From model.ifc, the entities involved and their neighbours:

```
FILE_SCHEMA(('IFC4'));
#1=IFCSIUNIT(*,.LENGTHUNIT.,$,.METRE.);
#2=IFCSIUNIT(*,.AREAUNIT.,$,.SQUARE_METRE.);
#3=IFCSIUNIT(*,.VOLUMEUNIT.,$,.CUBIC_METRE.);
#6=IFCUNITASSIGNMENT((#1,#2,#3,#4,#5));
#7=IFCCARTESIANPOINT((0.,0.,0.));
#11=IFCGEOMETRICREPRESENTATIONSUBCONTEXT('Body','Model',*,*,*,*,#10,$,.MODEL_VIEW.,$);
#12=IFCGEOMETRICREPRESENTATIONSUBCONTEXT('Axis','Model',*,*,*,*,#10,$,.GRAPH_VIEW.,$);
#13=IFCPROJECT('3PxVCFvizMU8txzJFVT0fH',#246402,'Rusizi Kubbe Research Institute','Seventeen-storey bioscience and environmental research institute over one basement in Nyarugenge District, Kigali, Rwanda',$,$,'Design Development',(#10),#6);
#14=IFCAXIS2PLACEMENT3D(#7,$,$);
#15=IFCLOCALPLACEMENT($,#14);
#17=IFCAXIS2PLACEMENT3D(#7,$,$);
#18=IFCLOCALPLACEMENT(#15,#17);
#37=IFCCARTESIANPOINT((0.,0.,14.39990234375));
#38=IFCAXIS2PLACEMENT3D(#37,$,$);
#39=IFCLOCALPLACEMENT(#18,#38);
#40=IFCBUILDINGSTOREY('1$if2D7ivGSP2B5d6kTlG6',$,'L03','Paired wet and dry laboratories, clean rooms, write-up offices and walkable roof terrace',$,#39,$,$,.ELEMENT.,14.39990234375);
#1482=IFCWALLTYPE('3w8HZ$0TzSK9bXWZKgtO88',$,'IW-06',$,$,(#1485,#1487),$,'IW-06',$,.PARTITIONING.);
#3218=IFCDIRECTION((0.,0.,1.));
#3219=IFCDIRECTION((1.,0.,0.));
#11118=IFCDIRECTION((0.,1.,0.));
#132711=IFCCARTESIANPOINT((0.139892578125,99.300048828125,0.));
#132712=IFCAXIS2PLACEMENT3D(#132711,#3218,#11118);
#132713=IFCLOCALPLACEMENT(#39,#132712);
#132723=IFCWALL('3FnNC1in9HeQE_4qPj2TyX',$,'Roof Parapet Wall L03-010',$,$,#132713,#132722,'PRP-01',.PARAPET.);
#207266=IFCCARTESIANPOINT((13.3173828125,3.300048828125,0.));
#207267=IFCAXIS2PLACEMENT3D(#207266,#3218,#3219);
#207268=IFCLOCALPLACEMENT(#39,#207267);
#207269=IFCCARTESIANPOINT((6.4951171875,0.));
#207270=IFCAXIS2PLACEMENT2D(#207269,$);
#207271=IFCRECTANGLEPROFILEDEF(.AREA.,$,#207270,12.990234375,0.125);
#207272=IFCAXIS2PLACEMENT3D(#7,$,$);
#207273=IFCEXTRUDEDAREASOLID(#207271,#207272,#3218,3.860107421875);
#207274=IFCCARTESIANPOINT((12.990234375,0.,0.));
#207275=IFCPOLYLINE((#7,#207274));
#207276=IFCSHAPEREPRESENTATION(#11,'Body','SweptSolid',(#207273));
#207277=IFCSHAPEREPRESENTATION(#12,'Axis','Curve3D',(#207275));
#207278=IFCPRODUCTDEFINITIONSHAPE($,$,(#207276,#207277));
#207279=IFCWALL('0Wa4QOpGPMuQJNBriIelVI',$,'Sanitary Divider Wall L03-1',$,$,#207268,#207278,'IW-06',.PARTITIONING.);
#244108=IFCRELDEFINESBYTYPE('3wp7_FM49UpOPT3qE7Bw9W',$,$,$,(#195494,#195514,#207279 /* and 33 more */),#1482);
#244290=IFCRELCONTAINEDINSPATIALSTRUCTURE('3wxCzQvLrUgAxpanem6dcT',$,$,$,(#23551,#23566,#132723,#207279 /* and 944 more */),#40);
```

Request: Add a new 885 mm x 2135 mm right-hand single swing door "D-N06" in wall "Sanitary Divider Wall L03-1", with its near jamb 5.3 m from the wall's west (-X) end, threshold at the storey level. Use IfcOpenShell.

```python
import numpy as np
import ifcopenshell
import ifcopenshell.api.feature
import ifcopenshell.api.geometry
import ifcopenshell.api.root
import ifcopenshell.api.spatial
import ifcopenshell.geom
import ifcopenshell.util.element
import ifcopenshell.util.placement
import ifcopenshell.util.representation
import ifcopenshell.util.shape
import ifcopenshell.util.unit

model = ifcopenshell.open("model.ifc")
unit_scale = ifcopenshell.util.unit.calculate_unit_scale(model)
settings = ifcopenshell.geom.settings()


def volume(element):
    """Net volume in cubic metres, openings subtracted."""
    shape = ifcopenshell.geom.create_shape(settings, element)
    return ifcopenshell.util.shape.get_volume(shape.geometry)


wall = model.by_id(207279)
storey = ifcopenshell.util.element.get_container(wall, ifc_class="IfcBuildingStorey")
context = ifcopenshell.util.representation.get_context(model, "Model", "Body", "MODEL_VIEW")
before = volume(wall)

width, height, from_end, sill = 0.885, 2.135, 5.3, 0.0  # metres

# The wall runs along its own X axis, and the end named is its -X end.
wall_shape = ifcopenshell.geom.create_shape(settings, wall)
x, y, z = ifcopenshell.util.shape.get_vertices(wall_shape.geometry).T
start = x.min() + from_end
face, thickness = float(y.min()), float(y.max() - y.min())
wall_matrix = ifcopenshell.util.placement.get_local_placement(wall.ObjectPlacement)
level = ifcopenshell.util.placement.get_local_placement(storey.ObjectPlacement)[2, 3]


def in_wall(x, y):
    """Placement at x, y metres in the wall's axes, at sill height."""
    matrix = wall_matrix.copy()
    matrix[:, 3] = wall_matrix @ np.array([x / unit_scale, y / unit_scale, 0.0, 1.0])
    matrix[2, 3] = level + sill / unit_scale
    return matrix


# Opening: a box that overshoots both wall faces by 50 mm.
opening = ifcopenshell.api.root.create_entity(model, ifc_class="IfcOpeningElement", predefined_type="OPENING")
box = ifcopenshell.api.geometry.add_wall_representation(
    model, context=context, length=width, height=height, thickness=thickness + 0.1
)
ifcopenshell.api.geometry.assign_representation(model, product=opening, representation=box)
ifcopenshell.api.geometry.edit_object_placement(model, product=opening, matrix=in_wall(start, face - 0.05), is_si=False)
ifcopenshell.api.feature.add_feature(model, feature=opening, element=wall)

door = ifcopenshell.api.root.create_entity(model, ifc_class="IfcDoor", name="D-N06", predefined_type="DOOR")
door.OverallWidth, door.OverallHeight = width / unit_scale, height / unit_scale
door.OperationType = "SINGLE_SWING_RIGHT"
body = ifcopenshell.api.geometry.add_door_representation(
    model,
    context=context,
    overall_width=door.OverallWidth,
    overall_height=door.OverallHeight,
    operation_type="SINGLE_SWING_RIGHT",
    lining_properties={"LiningDepth": thickness / unit_scale, "ThresholdDepth": thickness / unit_scale},
)
ifcopenshell.api.geometry.assign_representation(model, product=door, representation=body)
ifcopenshell.api.spatial.assign_container(model, products=[door], relating_structure=storey)
ifcopenshell.api.feature.add_filling(model, opening=opening, element=door)

# The lining spans the wall, so the door starts at the wall face.
ifcopenshell.api.geometry.edit_object_placement(model, product=door, matrix=in_wall(start, face), is_si=False)

after = volume(wall)

print(f"wall volume {before:.3f} -> {after:.3f} m3")

model.write("model_edited.ifc")
```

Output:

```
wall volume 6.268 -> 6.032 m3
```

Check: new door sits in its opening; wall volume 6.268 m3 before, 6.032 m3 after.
